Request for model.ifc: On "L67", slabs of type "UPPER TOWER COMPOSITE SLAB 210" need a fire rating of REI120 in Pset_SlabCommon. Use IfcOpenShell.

First a look at what the model holds.

```python
import ifcopenshell
import ifcopenshell.util.element

model = ifcopenshell.open("model.ifc")
print(model.schema)
storey = next(s for s in model.by_type("IfcBuildingStorey") if s.Name == "L67")
slabs = [e for e in ifcopenshell.util.element.get_decomposition(storey) if e.is_a("IfcSlab")]
seen = {}
for e in slabs:
    element_type = ifcopenshell.util.element.get_type(e)
    key = (element_type.Name if element_type != e and element_type else None, ifcopenshell.util.element.get_pset(e, "Pset_SlabCommon", "FireRating"))
    seen[key] = seen.get(key, 0) + 1
for (name, value), count in sorted(seen.items(), key=str):
    print(count, "x", name, "|", value)
```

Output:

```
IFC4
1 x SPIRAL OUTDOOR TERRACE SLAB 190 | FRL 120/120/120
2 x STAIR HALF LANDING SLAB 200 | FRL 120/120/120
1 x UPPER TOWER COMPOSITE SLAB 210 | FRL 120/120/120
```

```python
import ifcopenshell
import ifcopenshell.api.pset
import ifcopenshell.util.element

model = ifcopenshell.open("model.ifc")

storey = next(s for s in model.by_type("IfcBuildingStorey") if s.Name == "L67")
slabs = [e for e in ifcopenshell.util.element.get_decomposition(storey) if e.is_a("IfcSlab")]

count = 0
for e in slabs:
    element_type = ifcopenshell.util.element.get_type(e)
    if element_type in (None, e) or element_type.Name != "UPPER TOWER COMPOSITE SLAB 210":
        continue
    # add_pset returns the element's existing set when there is one.
    pset = ifcopenshell.api.pset.add_pset(model, product=e, name="Pset_SlabCommon")
    ifcopenshell.api.pset.edit_pset(model, pset=pset, properties={"FireRating": "REI120"})
    count += 1

print(count, "slabs updated")

model.write("model_v2.ifc")
```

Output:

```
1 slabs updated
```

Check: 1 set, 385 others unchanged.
